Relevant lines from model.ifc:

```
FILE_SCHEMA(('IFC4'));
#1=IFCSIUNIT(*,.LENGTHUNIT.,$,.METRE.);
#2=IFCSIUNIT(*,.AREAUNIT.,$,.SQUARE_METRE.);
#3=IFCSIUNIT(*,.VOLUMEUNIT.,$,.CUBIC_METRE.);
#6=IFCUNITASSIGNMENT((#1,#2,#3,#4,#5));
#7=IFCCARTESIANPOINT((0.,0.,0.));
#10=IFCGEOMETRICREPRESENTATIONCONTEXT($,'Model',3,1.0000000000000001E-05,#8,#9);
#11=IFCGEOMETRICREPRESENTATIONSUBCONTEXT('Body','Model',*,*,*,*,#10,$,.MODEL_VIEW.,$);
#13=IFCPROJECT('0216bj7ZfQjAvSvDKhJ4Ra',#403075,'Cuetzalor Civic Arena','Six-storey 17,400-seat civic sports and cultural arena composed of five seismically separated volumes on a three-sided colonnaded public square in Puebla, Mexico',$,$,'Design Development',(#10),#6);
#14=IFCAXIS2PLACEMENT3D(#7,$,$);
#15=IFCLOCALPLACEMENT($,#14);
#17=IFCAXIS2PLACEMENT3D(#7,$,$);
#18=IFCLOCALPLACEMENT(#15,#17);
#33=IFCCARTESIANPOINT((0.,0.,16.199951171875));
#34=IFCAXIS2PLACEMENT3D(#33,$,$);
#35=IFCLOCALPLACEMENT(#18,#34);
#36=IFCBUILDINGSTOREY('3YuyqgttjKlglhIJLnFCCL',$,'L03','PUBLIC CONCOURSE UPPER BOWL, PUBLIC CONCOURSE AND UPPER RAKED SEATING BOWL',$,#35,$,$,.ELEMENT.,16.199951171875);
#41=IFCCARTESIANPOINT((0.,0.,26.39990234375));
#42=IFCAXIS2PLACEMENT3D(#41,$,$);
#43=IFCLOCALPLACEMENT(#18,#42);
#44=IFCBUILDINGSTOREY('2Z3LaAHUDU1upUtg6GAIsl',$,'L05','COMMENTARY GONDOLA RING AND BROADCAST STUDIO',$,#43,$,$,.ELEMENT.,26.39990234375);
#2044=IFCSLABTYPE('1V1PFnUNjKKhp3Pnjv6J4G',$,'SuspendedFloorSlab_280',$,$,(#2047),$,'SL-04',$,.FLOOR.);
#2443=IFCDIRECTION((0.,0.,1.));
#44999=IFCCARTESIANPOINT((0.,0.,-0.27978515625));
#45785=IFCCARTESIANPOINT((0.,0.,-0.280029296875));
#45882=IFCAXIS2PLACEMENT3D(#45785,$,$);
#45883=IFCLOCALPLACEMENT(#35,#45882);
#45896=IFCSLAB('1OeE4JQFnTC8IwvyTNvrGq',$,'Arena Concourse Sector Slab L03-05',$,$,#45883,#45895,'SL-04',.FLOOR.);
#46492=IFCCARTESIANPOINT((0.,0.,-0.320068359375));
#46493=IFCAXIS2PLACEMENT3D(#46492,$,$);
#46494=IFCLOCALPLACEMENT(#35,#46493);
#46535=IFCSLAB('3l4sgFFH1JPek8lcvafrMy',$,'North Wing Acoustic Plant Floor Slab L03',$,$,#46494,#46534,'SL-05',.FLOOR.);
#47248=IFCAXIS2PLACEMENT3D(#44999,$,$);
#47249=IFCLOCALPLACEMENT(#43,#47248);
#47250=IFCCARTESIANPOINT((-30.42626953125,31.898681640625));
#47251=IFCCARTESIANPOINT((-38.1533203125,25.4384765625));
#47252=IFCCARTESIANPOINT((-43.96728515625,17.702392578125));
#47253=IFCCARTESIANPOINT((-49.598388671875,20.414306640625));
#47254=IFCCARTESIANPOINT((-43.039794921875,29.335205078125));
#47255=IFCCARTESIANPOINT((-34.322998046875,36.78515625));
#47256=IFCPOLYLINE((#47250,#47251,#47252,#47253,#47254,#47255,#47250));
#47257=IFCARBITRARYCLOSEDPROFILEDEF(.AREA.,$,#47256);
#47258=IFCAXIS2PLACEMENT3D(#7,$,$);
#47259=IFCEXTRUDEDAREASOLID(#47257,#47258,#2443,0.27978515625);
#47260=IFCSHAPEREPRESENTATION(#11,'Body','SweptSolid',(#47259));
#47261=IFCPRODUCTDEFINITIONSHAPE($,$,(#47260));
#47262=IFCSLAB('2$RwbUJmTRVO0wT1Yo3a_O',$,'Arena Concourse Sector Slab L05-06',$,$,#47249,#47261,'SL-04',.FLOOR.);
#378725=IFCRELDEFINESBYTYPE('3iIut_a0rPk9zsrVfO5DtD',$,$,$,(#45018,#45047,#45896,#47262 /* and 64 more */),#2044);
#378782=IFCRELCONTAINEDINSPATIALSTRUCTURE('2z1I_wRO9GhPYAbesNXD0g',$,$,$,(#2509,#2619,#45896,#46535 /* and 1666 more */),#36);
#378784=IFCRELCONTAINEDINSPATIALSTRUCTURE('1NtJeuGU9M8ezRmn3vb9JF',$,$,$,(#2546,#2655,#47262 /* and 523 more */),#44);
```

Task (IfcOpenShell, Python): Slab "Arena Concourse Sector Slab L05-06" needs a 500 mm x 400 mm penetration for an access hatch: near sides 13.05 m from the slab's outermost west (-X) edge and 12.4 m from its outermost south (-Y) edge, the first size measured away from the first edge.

```python
import numpy as np
import ifcopenshell
import ifcopenshell.api.feature
import ifcopenshell.api.geometry
import ifcopenshell.api.root
import ifcopenshell.geom
import ifcopenshell.util.placement
import ifcopenshell.util.representation
import ifcopenshell.util.shape
import ifcopenshell.util.unit

model = ifcopenshell.open("model.ifc")
unit_scale = ifcopenshell.util.unit.calculate_unit_scale(model)
settings = ifcopenshell.geom.settings()


def volume(element):
    """Net volume in cubic metres, openings subtracted."""
    shape = ifcopenshell.geom.create_shape(settings, element)
    return ifcopenshell.util.shape.get_volume(shape.geometry)


slab = model.by_guid("2$RwbUJmTRVO0wT1Yo3a_O")
before = volume(slab)

# Extent in the slab's own axes, in metres. The edges named are its -X and -Y sides.
slab_shape = ifcopenshell.geom.create_shape(settings, slab)
vertices = ifcopenshell.util.shape.get_vertices(slab_shape.geometry)
x_min, y_min, bottom = vertices.min(axis=0)
top = vertices[:, 2].max()

opening = ifcopenshell.api.root.create_entity(model, ifc_class="IfcOpeningElement", name="Access hatch opening", predefined_type="OPENING")
context = ifcopenshell.util.representation.get_context(model, "Model", "Body", "MODEL_VIEW")
width, depth = 0.5, 0.4
outline = [(0.0, 0.0), (width, 0.0), (width, depth), (0.0, depth), (0.0, 0.0)]
# Overshoot both faces by 50 mm so the cut is clean.
shape = ifcopenshell.api.geometry.add_slab_representation(
    model, context=context, depth=top - bottom + 0.1, polyline=outline
)
ifcopenshell.api.geometry.assign_representation(model, product=opening, representation=shape)

matrix = ifcopenshell.util.placement.get_local_placement(slab.ObjectPlacement)
matrix[:, 3] = matrix @ np.append(np.array([x_min + 13.05, y_min + 12.4, bottom - 0.05]) / unit_scale, 1.0)
ifcopenshell.api.geometry.edit_object_placement(model, product=opening, matrix=matrix, is_si=False)
ifcopenshell.api.feature.add_feature(model, feature=opening, element=slab)

after = volume(slab)

print(f"slab volume {before:.3f} -> {after:.3f} m3")

model.write("model_v2.ifc")
```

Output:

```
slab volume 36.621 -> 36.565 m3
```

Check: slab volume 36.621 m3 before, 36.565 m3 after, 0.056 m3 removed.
